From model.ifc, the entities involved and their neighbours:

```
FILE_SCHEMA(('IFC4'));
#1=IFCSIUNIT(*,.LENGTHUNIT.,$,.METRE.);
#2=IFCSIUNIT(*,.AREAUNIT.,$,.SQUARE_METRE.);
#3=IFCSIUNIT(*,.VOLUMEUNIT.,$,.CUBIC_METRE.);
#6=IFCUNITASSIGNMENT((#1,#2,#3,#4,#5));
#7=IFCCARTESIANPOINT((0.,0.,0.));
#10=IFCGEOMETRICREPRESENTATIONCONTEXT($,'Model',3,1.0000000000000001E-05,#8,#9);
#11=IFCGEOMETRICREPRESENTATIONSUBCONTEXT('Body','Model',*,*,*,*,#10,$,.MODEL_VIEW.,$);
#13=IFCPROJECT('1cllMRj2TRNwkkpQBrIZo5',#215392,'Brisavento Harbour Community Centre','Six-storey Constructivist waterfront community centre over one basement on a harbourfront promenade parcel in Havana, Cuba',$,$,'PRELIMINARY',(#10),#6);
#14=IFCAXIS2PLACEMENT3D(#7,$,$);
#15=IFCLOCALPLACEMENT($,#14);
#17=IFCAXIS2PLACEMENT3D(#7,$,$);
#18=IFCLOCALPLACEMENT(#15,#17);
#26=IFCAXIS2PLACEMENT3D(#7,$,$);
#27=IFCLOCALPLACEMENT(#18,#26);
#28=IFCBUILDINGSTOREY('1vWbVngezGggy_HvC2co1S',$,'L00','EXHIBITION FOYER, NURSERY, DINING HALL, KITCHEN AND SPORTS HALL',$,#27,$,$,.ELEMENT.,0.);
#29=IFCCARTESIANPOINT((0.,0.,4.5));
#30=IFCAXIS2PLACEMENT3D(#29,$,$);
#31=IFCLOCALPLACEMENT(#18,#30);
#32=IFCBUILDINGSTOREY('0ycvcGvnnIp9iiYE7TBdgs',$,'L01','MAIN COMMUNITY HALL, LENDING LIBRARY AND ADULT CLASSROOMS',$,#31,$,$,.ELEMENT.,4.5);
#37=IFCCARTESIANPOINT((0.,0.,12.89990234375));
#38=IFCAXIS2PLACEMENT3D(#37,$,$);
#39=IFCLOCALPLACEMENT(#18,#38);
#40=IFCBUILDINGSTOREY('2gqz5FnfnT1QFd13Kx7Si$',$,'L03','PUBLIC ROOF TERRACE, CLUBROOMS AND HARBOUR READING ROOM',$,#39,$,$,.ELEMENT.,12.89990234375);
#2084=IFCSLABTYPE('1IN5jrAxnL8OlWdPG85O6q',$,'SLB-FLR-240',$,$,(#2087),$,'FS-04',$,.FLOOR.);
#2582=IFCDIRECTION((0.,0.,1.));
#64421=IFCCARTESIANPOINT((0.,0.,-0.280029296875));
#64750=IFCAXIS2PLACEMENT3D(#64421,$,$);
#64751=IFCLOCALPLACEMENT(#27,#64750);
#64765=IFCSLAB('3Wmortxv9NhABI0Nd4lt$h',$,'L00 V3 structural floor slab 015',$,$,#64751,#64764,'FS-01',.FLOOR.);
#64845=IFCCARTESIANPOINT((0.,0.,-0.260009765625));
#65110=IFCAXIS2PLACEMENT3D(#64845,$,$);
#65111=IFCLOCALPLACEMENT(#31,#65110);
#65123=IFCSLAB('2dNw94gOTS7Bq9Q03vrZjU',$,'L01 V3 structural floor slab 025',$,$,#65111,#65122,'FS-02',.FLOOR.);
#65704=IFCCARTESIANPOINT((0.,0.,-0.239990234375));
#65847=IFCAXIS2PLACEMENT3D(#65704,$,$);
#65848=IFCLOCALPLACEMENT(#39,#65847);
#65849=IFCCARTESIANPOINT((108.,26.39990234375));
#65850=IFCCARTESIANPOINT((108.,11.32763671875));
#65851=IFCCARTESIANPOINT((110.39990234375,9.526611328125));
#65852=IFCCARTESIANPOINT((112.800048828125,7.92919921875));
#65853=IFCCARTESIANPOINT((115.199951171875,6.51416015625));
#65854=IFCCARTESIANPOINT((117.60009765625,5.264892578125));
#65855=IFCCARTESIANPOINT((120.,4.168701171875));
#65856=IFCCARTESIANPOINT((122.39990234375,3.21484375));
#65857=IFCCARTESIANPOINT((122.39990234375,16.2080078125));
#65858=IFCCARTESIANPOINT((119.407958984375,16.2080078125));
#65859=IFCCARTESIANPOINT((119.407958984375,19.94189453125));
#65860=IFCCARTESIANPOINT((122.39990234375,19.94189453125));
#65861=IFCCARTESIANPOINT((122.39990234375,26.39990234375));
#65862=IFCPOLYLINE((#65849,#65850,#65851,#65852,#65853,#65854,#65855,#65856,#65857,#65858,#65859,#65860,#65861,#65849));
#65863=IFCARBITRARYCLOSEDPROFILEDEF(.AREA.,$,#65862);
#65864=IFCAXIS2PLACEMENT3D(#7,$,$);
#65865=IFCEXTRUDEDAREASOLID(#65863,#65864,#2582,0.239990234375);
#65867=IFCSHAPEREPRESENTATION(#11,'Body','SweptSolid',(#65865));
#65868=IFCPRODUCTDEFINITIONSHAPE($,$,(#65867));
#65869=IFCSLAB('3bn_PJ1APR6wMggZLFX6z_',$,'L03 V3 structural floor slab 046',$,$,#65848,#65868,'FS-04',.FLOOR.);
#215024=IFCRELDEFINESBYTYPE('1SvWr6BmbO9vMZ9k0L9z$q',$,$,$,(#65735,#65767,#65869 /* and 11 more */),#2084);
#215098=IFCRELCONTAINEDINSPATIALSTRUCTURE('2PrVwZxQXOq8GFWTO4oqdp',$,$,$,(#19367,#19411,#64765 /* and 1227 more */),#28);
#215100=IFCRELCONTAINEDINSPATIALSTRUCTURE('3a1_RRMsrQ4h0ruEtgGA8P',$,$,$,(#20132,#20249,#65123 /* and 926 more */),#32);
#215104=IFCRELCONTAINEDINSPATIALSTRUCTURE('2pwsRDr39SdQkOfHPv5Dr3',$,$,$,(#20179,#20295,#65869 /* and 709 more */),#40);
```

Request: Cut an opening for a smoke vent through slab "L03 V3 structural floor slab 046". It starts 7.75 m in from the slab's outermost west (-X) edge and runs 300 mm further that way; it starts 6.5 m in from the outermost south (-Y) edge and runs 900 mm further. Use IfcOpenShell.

```python
import numpy as np
import ifcopenshell
import ifcopenshell.api.feature
import ifcopenshell.api.geometry
import ifcopenshell.api.root
import ifcopenshell.geom
import ifcopenshell.util.placement
import ifcopenshell.util.representation
import ifcopenshell.util.shape
import ifcopenshell.util.unit

model = ifcopenshell.open("model.ifc")
unit_scale = ifcopenshell.util.unit.calculate_unit_scale(model)
settings = ifcopenshell.geom.settings()


def volume(element):
    """Net volume in cubic metres, openings subtracted."""
    shape = ifcopenshell.geom.create_shape(settings, element)
    return ifcopenshell.util.shape.get_volume(shape.geometry)


slab = model.by_id(65869)
before = volume(slab)

# Extent in the slab's own axes, in metres. The edges named are its -X and -Y sides.
slab_shape = ifcopenshell.geom.create_shape(settings, slab)
vertices = ifcopenshell.util.shape.get_vertices(slab_shape.geometry)
x_min, y_min, bottom = vertices.min(axis=0)
top = vertices[:, 2].max()

opening = ifcopenshell.api.root.create_entity(model, ifc_class="IfcOpeningElement", name="Smoke vent opening", predefined_type="OPENING")
context = ifcopenshell.util.representation.get_context(model, "Model", "Body", "MODEL_VIEW")
width, depth = 0.3, 0.9
outline = [(0.0, 0.0), (width, 0.0), (width, depth), (0.0, depth), (0.0, 0.0)]
# Overshoot both faces by 50 mm so the cut is clean.
shape = ifcopenshell.api.geometry.add_slab_representation(
    model, context=context, depth=top - bottom + 0.1, polyline=outline
)
ifcopenshell.api.geometry.assign_representation(model, product=opening, representation=shape)

matrix = ifcopenshell.util.placement.get_local_placement(slab.ObjectPlacement)
matrix[:, 3] = matrix @ np.append(np.array([x_min + 7.75, y_min + 6.5, bottom - 0.05]) / unit_scale, 1.0)
ifcopenshell.api.geometry.edit_object_placement(model, product=opening, matrix=matrix, is_si=False)
ifcopenshell.api.feature.add_feature(model, feature=opening, element=slab)

after = volume(slab)

print(f"slab volume {before:.3f} -> {after:.3f} m3")

model.write("model_updated.ifc")
```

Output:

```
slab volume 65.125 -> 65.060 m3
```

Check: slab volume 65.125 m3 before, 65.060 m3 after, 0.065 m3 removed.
